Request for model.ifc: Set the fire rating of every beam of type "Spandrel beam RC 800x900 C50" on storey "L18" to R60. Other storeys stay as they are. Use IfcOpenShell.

First a look at what the model holds.

```python
import ifcopenshell
import ifcopenshell.util.element

model = ifcopenshell.open("model.ifc")
print(model.schema)
storey = next(s for s in model.by_type("IfcBuildingStorey") if s.Name == "L18")
beams = [e for e in ifcopenshell.util.element.get_decomposition(storey) if e.is_a("IfcBeam")]
seen = {}
for e in beams:
    element_type = ifcopenshell.util.element.get_type(e)
    key = (element_type.Name if element_type != e and element_type else None, ifcopenshell.util.element.get_pset(e, "Pset_BeamCommon", "FireRating"))
    seen[key] = seen.get(key, 0) + 1
for (name, value), count in sorted(seen.items(), key=str):
    print(count, "x", name, "|", value)
```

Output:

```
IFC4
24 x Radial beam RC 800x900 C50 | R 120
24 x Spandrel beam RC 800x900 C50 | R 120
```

```python
import ifcopenshell
import ifcopenshell.api.pset
import ifcopenshell.util.element

model = ifcopenshell.open("model.ifc")

storey = next(s for s in model.by_type("IfcBuildingStorey") if s.Name == "L18")
beams = [e for e in ifcopenshell.util.element.get_decomposition(storey) if e.is_a("IfcBeam")]

count = 0
for e in beams:
    element_type = ifcopenshell.util.element.get_type(e)
    if element_type in (None, e) or element_type.Name != "Spandrel beam RC 800x900 C50":
        continue
    # add_pset returns the element's existing set when there is one.
    pset = ifcopenshell.api.pset.add_pset(model, product=e, name="Pset_BeamCommon")
    ifcopenshell.api.pset.edit_pset(model, pset=pset, properties={"FireRating": "R60"})
    count += 1

print(count, "beams updated")

model.write("model_v2.ifc")
```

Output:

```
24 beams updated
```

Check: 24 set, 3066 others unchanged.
